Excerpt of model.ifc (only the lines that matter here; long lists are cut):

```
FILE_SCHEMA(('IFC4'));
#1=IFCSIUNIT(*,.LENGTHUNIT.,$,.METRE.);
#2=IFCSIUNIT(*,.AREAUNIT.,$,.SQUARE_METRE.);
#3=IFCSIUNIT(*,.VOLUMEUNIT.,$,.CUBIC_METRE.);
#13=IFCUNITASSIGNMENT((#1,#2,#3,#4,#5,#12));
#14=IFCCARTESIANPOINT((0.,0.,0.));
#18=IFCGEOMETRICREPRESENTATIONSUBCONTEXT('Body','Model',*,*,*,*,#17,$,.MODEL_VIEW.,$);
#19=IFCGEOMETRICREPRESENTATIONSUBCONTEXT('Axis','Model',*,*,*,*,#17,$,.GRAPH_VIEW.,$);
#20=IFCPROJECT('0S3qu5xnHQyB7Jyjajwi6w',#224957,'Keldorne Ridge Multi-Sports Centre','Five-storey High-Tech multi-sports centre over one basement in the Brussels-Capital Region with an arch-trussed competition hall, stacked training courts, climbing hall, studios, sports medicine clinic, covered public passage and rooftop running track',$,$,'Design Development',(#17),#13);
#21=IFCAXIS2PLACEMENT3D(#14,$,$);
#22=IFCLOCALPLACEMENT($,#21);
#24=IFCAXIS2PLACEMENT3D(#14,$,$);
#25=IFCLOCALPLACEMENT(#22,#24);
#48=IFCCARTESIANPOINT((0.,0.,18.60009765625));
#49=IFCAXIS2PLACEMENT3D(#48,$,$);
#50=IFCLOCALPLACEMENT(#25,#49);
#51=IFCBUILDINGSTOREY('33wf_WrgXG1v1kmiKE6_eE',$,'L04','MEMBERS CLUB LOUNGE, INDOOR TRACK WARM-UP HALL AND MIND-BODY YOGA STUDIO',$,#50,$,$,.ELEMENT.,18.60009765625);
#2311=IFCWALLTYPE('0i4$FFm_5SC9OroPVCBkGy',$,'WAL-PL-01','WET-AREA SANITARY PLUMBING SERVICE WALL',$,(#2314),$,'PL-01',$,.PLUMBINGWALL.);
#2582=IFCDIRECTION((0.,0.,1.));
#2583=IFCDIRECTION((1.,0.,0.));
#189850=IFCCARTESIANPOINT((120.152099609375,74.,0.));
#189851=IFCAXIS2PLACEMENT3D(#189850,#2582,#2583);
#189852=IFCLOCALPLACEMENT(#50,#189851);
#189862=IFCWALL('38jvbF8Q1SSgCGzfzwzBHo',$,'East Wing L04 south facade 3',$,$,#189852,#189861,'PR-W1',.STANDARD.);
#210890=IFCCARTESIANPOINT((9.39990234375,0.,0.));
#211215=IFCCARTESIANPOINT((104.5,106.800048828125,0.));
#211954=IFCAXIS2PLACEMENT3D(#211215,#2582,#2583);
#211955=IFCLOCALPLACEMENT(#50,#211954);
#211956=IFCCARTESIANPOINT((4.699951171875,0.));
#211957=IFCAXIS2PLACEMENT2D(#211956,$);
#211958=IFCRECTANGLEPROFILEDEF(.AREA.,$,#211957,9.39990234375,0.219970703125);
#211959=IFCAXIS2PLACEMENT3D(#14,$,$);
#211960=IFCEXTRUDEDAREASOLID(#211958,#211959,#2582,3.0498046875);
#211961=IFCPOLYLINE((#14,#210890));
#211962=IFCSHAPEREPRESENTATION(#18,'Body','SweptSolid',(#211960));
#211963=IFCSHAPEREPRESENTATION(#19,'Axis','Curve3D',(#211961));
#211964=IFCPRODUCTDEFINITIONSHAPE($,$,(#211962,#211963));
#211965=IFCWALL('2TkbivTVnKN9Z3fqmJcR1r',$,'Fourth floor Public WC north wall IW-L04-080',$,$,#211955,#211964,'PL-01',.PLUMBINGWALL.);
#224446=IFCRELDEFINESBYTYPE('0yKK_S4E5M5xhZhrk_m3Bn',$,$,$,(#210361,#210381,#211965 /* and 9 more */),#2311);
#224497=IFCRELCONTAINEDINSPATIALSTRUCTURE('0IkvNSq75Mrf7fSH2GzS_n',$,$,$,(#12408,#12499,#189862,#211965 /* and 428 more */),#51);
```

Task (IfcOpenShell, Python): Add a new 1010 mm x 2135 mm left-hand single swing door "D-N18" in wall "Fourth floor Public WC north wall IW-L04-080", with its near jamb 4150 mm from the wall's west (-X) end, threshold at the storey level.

```python
import numpy as np
import ifcopenshell
import ifcopenshell.api.feature
import ifcopenshell.api.geometry
import ifcopenshell.api.root
import ifcopenshell.api.spatial
import ifcopenshell.geom
import ifcopenshell.util.element
import ifcopenshell.util.placement
import ifcopenshell.util.representation
import ifcopenshell.util.shape
import ifcopenshell.util.unit

model = ifcopenshell.open("model.ifc")
unit_scale = ifcopenshell.util.unit.calculate_unit_scale(model)
settings = ifcopenshell.geom.settings()


def volume(element):
    """Net volume in cubic metres, openings subtracted."""
    shape = ifcopenshell.geom.create_shape(settings, element)
    return ifcopenshell.util.shape.get_volume(shape.geometry)


wall = model.by_guid("2TkbivTVnKN9Z3fqmJcR1r")
storey = ifcopenshell.util.element.get_container(wall, ifc_class="IfcBuildingStorey")
context = ifcopenshell.util.representation.get_context(model, "Model", "Body", "MODEL_VIEW")
before = volume(wall)

width, height, from_end, sill = 1.01, 2.135, 4.15, 0.0  # metres

# The wall runs along its own X axis, and the end named is its -X end.
wall_shape = ifcopenshell.geom.create_shape(settings, wall)
x, y, z = ifcopenshell.util.shape.get_vertices(wall_shape.geometry).T
start = x.min() + from_end
face, thickness = float(y.min()), float(y.max() - y.min())
wall_matrix = ifcopenshell.util.placement.get_local_placement(wall.ObjectPlacement)
level = ifcopenshell.util.placement.get_local_placement(storey.ObjectPlacement)[2, 3]


def in_wall(x, y):
    """Placement at x, y metres in the wall's axes, at sill height."""
    matrix = wall_matrix.copy()
    matrix[:, 3] = wall_matrix @ np.array([x / unit_scale, y / unit_scale, 0.0, 1.0])
    matrix[2, 3] = level + sill / unit_scale
    return matrix


# Opening: a box that overshoots both wall faces by 50 mm.
opening = ifcopenshell.api.root.create_entity(model, ifc_class="IfcOpeningElement", predefined_type="OPENING")
box = ifcopenshell.api.geometry.add_wall_representation(
    model, context=context, length=width, height=height, thickness=thickness + 0.1
)
ifcopenshell.api.geometry.assign_representation(model, product=opening, representation=box)
ifcopenshell.api.geometry.edit_object_placement(model, product=opening, matrix=in_wall(start, face - 0.05), is_si=False)
ifcopenshell.api.feature.add_feature(model, feature=opening, element=wall)

door = ifcopenshell.api.root.create_entity(model, ifc_class="IfcDoor", name="D-N18", predefined_type="DOOR")
door.OverallWidth, door.OverallHeight = width / unit_scale, height / unit_scale
door.OperationType = "SINGLE_SWING_LEFT"
body = ifcopenshell.api.geometry.add_door_representation(
    model,
    context=context,
    overall_width=door.OverallWidth,
    overall_height=door.OverallHeight,
    operation_type="SINGLE_SWING_LEFT",
    lining_properties={"LiningDepth": thickness / unit_scale, "ThresholdDepth": thickness / unit_scale},
)
ifcopenshell.api.geometry.assign_representation(model, product=door, representation=body)
ifcopenshell.api.spatial.assign_container(model, products=[door], relating_structure=storey)
ifcopenshell.api.feature.add_filling(model, opening=opening, element=door)

# The lining spans the wall, so the door starts at the wall face.
ifcopenshell.api.geometry.edit_object_placement(model, product=door, matrix=in_wall(start, face), is_si=False)

after = volume(wall)

print(f"wall volume {before:.3f} -> {after:.3f} m3")

model.write("model_v2.ifc")
```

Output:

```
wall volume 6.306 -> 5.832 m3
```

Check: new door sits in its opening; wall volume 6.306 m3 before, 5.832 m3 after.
